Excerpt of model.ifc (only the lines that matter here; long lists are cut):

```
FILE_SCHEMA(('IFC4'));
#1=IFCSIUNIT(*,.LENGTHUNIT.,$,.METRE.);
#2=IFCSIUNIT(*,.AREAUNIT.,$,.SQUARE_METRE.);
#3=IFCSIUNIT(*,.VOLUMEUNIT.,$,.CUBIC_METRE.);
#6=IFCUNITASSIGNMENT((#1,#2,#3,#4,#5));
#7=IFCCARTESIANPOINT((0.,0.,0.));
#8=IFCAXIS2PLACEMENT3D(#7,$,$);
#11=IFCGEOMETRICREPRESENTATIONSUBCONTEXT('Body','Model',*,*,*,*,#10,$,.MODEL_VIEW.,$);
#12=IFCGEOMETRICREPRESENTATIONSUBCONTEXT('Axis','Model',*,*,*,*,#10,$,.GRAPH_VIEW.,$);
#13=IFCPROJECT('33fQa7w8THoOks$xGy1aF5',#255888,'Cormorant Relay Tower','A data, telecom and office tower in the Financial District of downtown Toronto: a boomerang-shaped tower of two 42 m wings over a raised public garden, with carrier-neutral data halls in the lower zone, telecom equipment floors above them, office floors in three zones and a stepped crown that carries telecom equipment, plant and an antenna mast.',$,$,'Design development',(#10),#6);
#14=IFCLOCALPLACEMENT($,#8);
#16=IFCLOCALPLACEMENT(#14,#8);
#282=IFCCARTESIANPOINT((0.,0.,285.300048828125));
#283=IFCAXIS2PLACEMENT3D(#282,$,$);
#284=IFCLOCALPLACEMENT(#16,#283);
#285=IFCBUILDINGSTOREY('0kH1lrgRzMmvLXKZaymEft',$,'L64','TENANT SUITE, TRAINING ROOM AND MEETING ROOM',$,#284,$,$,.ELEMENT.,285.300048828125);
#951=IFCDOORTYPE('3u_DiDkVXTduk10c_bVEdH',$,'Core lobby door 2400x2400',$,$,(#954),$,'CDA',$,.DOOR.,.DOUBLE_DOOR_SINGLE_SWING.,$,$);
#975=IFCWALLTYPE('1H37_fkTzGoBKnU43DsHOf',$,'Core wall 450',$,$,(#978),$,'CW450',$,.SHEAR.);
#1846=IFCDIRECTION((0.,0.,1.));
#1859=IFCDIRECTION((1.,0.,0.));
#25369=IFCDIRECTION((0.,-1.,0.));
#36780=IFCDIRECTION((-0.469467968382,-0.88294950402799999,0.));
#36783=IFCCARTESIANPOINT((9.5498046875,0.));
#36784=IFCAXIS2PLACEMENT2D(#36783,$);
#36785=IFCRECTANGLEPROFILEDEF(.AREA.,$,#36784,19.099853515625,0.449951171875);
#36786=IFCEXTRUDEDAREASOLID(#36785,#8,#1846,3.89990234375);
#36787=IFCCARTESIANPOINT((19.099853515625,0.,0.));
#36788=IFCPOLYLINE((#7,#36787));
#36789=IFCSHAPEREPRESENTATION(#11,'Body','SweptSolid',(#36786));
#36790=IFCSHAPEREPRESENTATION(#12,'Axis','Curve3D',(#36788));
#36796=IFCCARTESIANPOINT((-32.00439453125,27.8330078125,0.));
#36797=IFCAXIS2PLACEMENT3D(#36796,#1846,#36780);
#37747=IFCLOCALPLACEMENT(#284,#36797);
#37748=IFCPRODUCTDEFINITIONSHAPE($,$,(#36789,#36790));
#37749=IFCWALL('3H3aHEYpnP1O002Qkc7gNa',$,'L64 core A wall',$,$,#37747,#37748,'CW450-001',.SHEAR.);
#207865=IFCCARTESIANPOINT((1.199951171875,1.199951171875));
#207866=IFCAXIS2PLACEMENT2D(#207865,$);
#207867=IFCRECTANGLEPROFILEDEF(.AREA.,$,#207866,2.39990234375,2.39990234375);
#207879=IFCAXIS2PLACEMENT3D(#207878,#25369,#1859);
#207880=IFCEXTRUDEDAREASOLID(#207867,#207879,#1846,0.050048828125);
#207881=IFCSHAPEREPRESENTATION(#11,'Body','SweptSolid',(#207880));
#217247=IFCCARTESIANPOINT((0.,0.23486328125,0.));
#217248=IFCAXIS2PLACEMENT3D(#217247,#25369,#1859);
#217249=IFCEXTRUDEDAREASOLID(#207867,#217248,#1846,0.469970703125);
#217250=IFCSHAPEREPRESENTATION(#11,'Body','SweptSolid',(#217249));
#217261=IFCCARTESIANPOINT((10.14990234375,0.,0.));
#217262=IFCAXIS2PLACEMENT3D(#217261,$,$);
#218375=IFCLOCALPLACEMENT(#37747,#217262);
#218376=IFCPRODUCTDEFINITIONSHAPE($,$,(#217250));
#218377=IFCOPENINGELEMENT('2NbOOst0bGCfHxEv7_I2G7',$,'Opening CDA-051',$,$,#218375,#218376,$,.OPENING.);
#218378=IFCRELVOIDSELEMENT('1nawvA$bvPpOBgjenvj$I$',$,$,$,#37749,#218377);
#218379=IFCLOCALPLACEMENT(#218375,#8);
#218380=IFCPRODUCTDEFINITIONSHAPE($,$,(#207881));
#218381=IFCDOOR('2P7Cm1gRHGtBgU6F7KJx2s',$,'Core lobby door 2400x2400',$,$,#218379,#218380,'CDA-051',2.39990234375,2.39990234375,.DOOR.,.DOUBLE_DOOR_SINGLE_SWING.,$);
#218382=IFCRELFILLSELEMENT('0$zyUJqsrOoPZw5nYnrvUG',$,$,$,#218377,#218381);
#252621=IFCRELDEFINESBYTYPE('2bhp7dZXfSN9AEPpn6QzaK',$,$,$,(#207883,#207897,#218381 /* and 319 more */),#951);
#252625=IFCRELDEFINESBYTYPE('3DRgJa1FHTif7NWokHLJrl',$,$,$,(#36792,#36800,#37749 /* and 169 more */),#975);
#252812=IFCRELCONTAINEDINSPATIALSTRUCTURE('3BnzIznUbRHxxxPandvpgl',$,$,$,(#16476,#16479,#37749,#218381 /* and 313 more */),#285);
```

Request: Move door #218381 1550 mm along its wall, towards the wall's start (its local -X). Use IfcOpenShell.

```python
import ifcopenshell
import ifcopenshell.api.geometry
import ifcopenshell.util.placement

model = ifcopenshell.open("model.ifc")

door = model.by_guid("2P7Cm1gRHGtBgU6F7KJx2s")
opening = door.FillsVoids[0].RelatingOpeningElement
wall = opening.VoidsElements[0].RelatingBuildingElement

wall_matrix = ifcopenshell.util.placement.get_local_placement(wall.ObjectPlacement)
shift = wall_matrix[:3, 0] * -1.55
before = ifcopenshell.util.placement.get_local_placement(door.ObjectPlacement)[:3, 3].copy()

# The door is placed relative to its opening, so it follows when the opening moves.
matrix = ifcopenshell.util.placement.get_local_placement(opening.ObjectPlacement)
matrix[:3, 3] += shift
ifcopenshell.api.geometry.edit_object_placement(
    model, product=opening, matrix=matrix, is_si=False, should_transform_children=True
)

after = ifcopenshell.util.placement.get_local_placement(door.ObjectPlacement)[:3, 3]
print("door moved by", (after - before).round(3) + 0.0)

model.write("model_edited.ifc")
```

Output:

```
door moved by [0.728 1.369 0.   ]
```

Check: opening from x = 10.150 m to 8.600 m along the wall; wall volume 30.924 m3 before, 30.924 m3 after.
